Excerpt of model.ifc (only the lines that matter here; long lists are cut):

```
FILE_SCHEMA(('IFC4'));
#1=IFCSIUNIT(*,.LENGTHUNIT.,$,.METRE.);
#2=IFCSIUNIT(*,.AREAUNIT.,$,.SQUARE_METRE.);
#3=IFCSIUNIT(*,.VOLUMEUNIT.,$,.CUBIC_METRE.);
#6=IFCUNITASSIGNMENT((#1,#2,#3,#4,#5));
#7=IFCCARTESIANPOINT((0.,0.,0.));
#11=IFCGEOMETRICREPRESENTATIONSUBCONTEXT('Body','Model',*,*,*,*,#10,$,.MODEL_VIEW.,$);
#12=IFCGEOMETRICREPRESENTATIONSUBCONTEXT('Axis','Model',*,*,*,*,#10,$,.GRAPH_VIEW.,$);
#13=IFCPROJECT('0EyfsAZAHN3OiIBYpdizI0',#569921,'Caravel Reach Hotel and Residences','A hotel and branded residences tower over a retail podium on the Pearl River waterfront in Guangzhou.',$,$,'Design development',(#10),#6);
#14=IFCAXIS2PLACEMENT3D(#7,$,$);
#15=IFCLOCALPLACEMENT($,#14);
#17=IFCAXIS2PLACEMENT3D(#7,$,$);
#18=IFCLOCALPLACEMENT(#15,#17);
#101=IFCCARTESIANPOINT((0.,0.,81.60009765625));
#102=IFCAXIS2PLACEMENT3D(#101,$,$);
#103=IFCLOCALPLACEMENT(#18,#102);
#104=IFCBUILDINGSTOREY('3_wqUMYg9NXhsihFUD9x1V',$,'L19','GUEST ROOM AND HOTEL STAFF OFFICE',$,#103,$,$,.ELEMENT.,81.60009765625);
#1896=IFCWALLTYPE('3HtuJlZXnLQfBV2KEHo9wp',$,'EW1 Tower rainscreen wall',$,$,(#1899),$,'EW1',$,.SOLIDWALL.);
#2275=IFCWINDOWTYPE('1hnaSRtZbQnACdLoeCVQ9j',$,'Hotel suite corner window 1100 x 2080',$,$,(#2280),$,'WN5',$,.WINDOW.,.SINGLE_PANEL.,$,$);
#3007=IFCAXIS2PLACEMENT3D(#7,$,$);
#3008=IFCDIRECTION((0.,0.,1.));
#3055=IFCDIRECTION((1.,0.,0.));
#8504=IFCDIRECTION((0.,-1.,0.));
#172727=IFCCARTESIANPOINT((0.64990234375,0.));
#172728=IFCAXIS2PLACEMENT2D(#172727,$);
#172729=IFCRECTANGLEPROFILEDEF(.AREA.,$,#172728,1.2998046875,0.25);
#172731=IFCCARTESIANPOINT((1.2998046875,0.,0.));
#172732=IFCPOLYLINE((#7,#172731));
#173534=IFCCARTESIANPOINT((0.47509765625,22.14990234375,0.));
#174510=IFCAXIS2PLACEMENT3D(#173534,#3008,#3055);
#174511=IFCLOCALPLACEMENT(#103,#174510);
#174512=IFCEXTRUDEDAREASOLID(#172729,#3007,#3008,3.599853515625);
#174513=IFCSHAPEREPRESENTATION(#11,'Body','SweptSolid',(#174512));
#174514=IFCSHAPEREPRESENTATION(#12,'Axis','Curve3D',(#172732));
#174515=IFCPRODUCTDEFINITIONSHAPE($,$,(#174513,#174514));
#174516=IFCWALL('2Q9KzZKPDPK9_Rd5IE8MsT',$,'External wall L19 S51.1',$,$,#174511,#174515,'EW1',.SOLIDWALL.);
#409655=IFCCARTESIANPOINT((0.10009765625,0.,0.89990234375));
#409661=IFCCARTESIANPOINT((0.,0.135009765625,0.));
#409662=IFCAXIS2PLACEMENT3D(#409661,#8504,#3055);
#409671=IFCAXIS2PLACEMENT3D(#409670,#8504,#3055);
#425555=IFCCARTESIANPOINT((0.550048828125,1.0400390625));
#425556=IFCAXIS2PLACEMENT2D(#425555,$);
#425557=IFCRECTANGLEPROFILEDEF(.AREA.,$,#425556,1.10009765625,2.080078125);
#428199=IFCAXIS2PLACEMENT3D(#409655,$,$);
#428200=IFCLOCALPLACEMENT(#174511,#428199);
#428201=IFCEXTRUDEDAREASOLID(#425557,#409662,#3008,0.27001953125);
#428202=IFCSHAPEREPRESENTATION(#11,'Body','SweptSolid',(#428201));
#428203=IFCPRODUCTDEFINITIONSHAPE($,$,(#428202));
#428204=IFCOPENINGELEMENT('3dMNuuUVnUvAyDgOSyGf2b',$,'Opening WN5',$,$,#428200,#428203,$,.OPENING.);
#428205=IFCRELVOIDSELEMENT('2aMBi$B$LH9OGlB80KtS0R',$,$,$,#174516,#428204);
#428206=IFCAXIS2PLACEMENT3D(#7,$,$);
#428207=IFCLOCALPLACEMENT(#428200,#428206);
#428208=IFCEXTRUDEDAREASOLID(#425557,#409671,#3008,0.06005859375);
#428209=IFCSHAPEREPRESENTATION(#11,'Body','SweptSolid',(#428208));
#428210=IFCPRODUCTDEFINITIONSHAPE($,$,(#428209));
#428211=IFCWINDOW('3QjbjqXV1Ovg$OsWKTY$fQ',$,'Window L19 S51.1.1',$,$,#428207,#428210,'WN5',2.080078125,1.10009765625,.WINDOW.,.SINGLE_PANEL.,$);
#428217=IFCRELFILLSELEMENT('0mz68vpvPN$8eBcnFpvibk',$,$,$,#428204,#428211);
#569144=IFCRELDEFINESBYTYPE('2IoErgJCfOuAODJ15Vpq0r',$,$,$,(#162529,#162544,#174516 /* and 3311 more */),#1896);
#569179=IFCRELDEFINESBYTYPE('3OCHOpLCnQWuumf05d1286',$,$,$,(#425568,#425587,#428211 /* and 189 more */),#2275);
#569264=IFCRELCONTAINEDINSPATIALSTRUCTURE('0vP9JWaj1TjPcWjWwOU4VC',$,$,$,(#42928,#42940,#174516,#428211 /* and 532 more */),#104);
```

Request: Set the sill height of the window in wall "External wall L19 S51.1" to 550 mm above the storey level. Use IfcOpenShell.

```python
import numpy as np
import ifcopenshell
import ifcopenshell.api.geometry
import ifcopenshell.geom
import ifcopenshell.util.element
import ifcopenshell.util.placement
import ifcopenshell.util.shape
import ifcopenshell.util.unit

model = ifcopenshell.open("model.ifc")
unit_scale = ifcopenshell.util.unit.calculate_unit_scale(model)

window = model.by_id(428211)
opening = window.FillsVoids[0].RelatingOpeningElement
storey = ifcopenshell.util.element.get_container(window, ifc_class="IfcBuildingStorey")
level = ifcopenshell.util.placement.get_local_placement(storey.ObjectPlacement)[2, 3]

# The opening's origin need not be at the sill, so measure its lowest point.
shape = ifcopenshell.geom.create_shape(ifcopenshell.geom.settings(), opening)
bottom = ifcopenshell.util.shape.get_shape_bottom_elevation(shape, shape.geometry) / unit_scale
dz = level + 0.55 - bottom

shift = np.array([0.0, 0.0, dz])
# The window is placed relative to its opening, so it follows when the opening moves.
matrix = ifcopenshell.util.placement.get_local_placement(opening.ObjectPlacement)
matrix[:3, 3] += shift
ifcopenshell.api.geometry.edit_object_placement(
    model, product=opening, matrix=matrix, is_si=False, should_transform_children=True
)

print(f"moved by {dz * unit_scale:+.3f} m")

model.write("model_rev.ifc")
```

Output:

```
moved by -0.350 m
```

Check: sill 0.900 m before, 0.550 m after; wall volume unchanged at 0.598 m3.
